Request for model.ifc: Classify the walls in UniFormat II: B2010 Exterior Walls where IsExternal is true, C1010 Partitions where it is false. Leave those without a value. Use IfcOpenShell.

First a look at what the model holds.

```python
import ifcopenshell
import ifcopenshell.util.element

model = ifcopenshell.open("model.ifc")
print(model.schema)
print("classifications:", [c.Name for c in model.by_type("IfcClassification")])
values = [ifcopenshell.util.element.get_pset(e, "Pset_WallCommon", "IsExternal") for e in model.by_type("IfcWall")]
for value in (True, False, None):
    print("IsExternal", value, values.count(value))
```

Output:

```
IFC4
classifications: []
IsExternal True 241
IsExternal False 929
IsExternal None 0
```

```python
import ifcopenshell
import ifcopenshell.api.classification
import ifcopenshell.util.element

model = ifcopenshell.open("model.ifc")

system = ifcopenshell.api.classification.add_classification(model, classification="UniFormat II")

walls = model.by_type("IfcWall")
external = {e: ifcopenshell.util.element.get_pset(e, "Pset_WallCommon", "IsExternal") for e in walls}
for flag, code, name in ((True, "B2010", "Exterior Walls"), (False, "C1010", "Partitions")):
    products = [e for e in walls if external[e] is flag]
    ifcopenshell.api.classification.add_reference(
        model, products=products, classification=system, identification=code, name=name
    )
    print(code, len(products))

model.write("model_updated.ifc")
```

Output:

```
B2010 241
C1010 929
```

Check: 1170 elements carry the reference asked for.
